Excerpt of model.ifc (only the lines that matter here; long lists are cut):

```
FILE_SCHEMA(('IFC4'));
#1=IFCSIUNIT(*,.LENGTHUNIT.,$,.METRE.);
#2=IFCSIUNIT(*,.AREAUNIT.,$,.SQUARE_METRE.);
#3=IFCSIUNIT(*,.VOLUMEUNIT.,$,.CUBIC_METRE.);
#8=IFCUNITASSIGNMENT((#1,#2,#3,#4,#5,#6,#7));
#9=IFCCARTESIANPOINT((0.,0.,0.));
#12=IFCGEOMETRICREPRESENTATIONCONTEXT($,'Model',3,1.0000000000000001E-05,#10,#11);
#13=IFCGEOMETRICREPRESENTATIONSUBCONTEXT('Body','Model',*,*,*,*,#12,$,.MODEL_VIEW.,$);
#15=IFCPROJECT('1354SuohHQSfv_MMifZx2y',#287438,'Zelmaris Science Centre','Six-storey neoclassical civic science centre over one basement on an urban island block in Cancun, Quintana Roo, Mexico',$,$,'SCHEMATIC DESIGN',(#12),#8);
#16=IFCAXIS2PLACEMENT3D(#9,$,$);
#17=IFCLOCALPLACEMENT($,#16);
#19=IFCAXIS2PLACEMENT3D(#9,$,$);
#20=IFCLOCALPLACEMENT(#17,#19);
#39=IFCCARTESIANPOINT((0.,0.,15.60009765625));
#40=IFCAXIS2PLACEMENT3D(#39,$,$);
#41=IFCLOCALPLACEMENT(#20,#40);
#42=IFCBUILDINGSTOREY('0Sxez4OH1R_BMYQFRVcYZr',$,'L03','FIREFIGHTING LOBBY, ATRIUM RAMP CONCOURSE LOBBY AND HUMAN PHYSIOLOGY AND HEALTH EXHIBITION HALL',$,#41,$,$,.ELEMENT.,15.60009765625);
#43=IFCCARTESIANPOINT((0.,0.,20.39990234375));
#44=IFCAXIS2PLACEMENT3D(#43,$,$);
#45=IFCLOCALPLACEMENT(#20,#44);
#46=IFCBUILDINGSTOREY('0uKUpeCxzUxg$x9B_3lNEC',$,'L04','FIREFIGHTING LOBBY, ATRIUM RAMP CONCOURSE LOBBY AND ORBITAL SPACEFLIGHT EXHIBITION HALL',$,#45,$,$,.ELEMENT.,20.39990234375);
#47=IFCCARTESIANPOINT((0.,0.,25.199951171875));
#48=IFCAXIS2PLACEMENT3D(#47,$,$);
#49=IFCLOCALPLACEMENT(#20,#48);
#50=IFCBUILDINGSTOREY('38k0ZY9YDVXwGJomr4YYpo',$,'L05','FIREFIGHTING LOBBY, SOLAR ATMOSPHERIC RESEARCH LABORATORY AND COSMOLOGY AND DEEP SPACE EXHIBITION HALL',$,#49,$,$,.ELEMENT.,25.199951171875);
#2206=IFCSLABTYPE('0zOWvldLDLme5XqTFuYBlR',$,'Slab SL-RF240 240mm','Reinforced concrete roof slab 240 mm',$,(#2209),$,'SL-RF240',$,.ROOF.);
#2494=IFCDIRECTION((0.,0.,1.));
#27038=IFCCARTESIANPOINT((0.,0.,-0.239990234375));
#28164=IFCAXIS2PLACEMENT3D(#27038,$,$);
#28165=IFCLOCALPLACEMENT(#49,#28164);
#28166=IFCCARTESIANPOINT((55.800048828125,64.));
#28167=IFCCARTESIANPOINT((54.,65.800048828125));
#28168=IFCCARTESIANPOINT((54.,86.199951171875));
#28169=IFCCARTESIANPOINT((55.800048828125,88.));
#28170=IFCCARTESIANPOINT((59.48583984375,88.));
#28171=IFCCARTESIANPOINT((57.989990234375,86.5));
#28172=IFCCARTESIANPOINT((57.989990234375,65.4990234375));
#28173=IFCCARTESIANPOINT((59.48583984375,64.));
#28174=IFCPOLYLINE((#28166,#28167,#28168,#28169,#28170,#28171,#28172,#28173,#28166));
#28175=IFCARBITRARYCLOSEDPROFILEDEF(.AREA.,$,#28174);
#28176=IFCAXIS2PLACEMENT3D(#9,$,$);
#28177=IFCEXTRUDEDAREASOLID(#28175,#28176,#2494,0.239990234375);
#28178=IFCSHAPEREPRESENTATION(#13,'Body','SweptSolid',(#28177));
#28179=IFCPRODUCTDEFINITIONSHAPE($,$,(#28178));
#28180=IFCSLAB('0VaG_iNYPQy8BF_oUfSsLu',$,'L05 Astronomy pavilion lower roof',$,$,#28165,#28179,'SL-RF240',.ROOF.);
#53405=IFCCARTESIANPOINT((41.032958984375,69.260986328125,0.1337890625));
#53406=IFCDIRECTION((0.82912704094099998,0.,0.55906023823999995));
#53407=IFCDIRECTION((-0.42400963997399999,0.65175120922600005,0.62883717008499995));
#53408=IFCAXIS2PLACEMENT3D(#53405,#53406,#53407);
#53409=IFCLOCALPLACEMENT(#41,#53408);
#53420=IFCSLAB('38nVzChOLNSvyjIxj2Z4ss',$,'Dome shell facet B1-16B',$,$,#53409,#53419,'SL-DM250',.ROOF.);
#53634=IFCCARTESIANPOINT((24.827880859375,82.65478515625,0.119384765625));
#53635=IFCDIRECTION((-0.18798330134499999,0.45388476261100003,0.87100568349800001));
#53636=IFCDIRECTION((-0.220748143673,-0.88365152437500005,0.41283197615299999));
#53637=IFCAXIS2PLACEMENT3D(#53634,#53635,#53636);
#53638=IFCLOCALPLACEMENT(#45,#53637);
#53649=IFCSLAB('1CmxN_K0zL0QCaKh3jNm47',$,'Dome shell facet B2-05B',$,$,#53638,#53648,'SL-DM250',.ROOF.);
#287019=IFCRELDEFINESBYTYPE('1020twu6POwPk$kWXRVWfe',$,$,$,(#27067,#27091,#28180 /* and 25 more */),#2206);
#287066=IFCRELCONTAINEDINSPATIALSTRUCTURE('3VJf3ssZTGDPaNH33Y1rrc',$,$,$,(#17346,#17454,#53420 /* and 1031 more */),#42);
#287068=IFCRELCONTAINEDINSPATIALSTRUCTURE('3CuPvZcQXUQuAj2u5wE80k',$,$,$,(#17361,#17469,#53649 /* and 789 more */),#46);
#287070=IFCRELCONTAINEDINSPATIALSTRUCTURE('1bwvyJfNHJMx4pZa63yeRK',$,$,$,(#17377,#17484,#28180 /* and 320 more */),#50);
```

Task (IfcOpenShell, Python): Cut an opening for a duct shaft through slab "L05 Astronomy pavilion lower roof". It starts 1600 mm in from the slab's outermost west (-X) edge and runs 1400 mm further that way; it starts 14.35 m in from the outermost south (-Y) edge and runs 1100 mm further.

```python
import numpy as np
import ifcopenshell
import ifcopenshell.api.feature
import ifcopenshell.api.geometry
import ifcopenshell.api.root
import ifcopenshell.geom
import ifcopenshell.util.placement
import ifcopenshell.util.representation
import ifcopenshell.util.shape
import ifcopenshell.util.unit

model = ifcopenshell.open("model.ifc")
unit_scale = ifcopenshell.util.unit.calculate_unit_scale(model)
settings = ifcopenshell.geom.settings()


def volume(element):
    """Net volume in cubic metres, openings subtracted."""
    shape = ifcopenshell.geom.create_shape(settings, element)
    return ifcopenshell.util.shape.get_volume(shape.geometry)


slab = model.by_guid("0VaG_iNYPQy8BF_oUfSsLu")
before = volume(slab)

# Extent in the slab's own axes, in metres. The edges named are its -X and -Y sides.
slab_shape = ifcopenshell.geom.create_shape(settings, slab)
vertices = ifcopenshell.util.shape.get_vertices(slab_shape.geometry)
x_min, y_min, bottom = vertices.min(axis=0)
top = vertices[:, 2].max()

opening = ifcopenshell.api.root.create_entity(model, ifc_class="IfcOpeningElement", name="Duct shaft opening", predefined_type="OPENING")
context = ifcopenshell.util.representation.get_context(model, "Model", "Body", "MODEL_VIEW")
width, depth = 1.4, 1.1
outline = [(0.0, 0.0), (width, 0.0), (width, depth), (0.0, depth), (0.0, 0.0)]
# Overshoot both faces by 50 mm so the cut is clean.
shape = ifcopenshell.api.geometry.add_slab_representation(
    model, context=context, depth=top - bottom + 0.1, polyline=outline
)
ifcopenshell.api.geometry.assign_representation(model, product=opening, representation=shape)

matrix = ifcopenshell.util.placement.get_local_placement(slab.ObjectPlacement)
matrix[:, 3] = matrix @ np.append(np.array([x_min + 1.6, y_min + 14.35, bottom - 0.05]) / unit_scale, 1.0)
ifcopenshell.api.geometry.edit_object_placement(model, product=opening, matrix=matrix, is_si=False)
ifcopenshell.api.feature.add_feature(model, feature=opening, element=slab)

after = volume(slab)

print(f"slab volume {before:.3f} -> {after:.3f} m3")

model.write("model_edited.ifc")
```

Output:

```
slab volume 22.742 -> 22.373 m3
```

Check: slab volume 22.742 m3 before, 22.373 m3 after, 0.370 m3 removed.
